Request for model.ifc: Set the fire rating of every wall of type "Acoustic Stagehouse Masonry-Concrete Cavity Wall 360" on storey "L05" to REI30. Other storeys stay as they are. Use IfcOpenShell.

First a look at what the model holds.

```python
import ifcopenshell
import ifcopenshell.util.element

model = ifcopenshell.open("model.ifc")
print(model.schema)
storey = next(s for s in model.by_type("IfcBuildingStorey") if s.Name == "L05")
walls = [e for e in ifcopenshell.util.element.get_decomposition(storey) if e.is_a("IfcWall")]
seen = {}
for e in walls:
    element_type = ifcopenshell.util.element.get_type(e)
    key = (element_type.Name if element_type != e and element_type else None, ifcopenshell.util.element.get_pset(e, "Pset_WallCommon", "FireRating"))
    seen[key] = seen.get(key, 0) + 1
for (name, value), count in sorted(seen.items(), key=str):
    print(count, "x", name, "|", value)
```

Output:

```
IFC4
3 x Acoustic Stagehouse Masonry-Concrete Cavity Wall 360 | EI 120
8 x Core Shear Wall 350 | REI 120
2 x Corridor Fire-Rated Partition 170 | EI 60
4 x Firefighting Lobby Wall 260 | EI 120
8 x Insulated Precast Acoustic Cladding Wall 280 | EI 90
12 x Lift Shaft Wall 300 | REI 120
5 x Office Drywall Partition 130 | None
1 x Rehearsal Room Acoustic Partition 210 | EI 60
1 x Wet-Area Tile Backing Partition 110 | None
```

```python
import ifcopenshell
import ifcopenshell.api.pset
import ifcopenshell.util.element

model = ifcopenshell.open("model.ifc")

storey = next(s for s in model.by_type("IfcBuildingStorey") if s.Name == "L05")
walls = [e for e in ifcopenshell.util.element.get_decomposition(storey) if e.is_a("IfcWall")]

count = 0
for e in walls:
    element_type = ifcopenshell.util.element.get_type(e)
    if element_type in (None, e) or element_type.Name != "Acoustic Stagehouse Masonry-Concrete Cavity Wall 360":
        continue
    # add_pset returns the element's existing set when there is one.
    pset = ifcopenshell.api.pset.add_pset(model, product=e, name="Pset_WallCommon")
    ifcopenshell.api.pset.edit_pset(model, pset=pset, properties={"FireRating": "REI30"})
    count += 1

print(count, "walls updated")

model.write("model_v2.ifc")
```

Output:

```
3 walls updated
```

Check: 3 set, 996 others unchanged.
